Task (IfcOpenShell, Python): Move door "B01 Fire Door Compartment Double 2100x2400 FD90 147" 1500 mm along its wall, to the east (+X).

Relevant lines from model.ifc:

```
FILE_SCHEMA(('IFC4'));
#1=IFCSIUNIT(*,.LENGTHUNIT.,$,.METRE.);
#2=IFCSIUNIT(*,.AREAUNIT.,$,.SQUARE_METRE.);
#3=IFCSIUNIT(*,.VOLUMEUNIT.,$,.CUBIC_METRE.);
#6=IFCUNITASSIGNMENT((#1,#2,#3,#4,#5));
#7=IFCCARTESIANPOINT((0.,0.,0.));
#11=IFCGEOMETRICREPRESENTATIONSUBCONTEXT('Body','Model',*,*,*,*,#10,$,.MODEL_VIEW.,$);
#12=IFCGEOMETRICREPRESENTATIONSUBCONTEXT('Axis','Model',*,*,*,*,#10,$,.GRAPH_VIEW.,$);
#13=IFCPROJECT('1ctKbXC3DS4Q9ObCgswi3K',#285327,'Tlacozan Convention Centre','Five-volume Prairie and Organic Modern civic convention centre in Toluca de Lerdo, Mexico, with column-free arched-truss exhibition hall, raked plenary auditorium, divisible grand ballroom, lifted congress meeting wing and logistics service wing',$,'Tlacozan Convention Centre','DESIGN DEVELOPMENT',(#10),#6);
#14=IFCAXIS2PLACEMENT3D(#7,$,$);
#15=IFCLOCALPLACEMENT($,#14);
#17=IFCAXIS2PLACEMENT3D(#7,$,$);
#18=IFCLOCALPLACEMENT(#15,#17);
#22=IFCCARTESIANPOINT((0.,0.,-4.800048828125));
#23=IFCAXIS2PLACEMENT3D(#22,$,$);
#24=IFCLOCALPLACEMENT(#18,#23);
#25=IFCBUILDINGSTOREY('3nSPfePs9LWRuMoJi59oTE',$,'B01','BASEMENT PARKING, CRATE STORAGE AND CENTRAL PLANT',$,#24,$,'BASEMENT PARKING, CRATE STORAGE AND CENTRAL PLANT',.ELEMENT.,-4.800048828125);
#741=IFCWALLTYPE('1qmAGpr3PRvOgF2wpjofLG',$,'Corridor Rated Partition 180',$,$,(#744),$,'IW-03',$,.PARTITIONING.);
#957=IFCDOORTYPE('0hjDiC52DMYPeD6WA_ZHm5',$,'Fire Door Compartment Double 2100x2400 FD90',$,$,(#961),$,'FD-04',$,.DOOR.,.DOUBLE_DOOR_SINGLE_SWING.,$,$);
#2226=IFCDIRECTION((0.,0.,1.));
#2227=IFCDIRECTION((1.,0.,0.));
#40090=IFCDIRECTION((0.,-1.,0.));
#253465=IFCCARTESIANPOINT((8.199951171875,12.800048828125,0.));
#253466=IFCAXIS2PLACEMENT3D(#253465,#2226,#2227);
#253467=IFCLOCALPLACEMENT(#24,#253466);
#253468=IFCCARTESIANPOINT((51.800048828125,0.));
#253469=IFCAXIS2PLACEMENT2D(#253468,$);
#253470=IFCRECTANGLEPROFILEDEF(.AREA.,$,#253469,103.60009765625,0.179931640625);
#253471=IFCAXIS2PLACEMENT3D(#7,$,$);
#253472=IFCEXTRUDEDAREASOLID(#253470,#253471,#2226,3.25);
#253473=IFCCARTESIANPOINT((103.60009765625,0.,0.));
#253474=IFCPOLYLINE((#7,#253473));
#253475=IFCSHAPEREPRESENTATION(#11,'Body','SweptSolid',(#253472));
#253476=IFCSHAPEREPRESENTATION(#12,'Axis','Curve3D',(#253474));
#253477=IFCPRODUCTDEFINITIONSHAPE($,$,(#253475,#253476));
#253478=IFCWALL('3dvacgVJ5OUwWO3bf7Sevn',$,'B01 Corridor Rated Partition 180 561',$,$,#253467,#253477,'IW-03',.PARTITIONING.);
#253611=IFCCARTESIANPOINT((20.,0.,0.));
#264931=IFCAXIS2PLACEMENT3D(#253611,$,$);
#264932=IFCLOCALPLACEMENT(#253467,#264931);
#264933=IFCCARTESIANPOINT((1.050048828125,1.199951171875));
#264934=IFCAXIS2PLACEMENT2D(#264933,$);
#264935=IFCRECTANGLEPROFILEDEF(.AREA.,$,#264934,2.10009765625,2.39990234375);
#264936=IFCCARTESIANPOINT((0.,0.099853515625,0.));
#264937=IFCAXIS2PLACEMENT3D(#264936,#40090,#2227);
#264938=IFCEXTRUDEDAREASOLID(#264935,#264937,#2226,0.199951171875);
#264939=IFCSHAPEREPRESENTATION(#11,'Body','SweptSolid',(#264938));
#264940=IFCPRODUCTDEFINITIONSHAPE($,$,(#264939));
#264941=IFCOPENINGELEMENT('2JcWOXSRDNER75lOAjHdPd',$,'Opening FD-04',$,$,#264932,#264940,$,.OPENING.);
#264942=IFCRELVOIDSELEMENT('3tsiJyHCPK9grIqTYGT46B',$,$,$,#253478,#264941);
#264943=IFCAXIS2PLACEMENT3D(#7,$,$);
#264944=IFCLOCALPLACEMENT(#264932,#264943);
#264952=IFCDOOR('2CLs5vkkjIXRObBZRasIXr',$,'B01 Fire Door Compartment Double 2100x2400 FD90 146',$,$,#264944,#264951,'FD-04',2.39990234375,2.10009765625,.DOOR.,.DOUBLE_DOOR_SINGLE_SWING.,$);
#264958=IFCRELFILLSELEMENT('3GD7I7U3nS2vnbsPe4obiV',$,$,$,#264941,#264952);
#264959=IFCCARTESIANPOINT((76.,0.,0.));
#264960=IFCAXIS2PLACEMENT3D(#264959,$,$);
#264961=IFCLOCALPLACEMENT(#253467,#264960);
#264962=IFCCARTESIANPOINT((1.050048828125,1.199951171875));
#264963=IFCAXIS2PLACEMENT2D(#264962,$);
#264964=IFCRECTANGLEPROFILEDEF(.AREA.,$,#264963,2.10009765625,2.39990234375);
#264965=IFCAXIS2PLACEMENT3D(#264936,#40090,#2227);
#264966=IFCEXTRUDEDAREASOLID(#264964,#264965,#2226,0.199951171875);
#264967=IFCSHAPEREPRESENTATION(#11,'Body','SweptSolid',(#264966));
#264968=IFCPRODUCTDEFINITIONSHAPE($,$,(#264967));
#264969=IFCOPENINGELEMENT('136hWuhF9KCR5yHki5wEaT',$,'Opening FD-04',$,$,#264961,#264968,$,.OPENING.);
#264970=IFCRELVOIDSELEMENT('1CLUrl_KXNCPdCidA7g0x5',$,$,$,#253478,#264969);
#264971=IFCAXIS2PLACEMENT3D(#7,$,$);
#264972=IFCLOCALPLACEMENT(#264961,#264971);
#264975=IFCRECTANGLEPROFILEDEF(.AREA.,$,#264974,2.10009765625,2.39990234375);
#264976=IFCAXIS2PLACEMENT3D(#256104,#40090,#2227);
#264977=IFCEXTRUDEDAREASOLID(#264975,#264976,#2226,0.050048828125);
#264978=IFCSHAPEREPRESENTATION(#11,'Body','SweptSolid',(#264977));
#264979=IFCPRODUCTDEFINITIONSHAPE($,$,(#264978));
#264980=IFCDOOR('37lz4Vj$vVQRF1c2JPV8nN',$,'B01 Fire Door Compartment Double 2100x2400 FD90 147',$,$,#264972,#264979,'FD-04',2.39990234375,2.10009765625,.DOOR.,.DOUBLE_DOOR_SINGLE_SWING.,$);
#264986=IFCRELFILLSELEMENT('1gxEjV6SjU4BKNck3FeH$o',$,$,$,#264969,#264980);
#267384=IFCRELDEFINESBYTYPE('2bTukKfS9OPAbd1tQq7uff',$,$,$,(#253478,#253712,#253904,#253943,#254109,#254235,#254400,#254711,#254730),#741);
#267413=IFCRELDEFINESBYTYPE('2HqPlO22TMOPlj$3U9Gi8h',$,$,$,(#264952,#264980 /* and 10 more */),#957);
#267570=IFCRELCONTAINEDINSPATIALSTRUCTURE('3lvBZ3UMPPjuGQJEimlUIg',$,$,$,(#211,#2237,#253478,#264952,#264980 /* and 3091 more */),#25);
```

```python
import ifcopenshell
import ifcopenshell.api.geometry
import ifcopenshell.util.placement
import ifcopenshell.util.unit

model = ifcopenshell.open("model.ifc")
unit_scale = ifcopenshell.util.unit.calculate_unit_scale(model)

door = model.by_guid("37lz4Vj$vVQRF1c2JPV8nN")
opening = door.FillsVoids[0].RelatingOpeningElement
wall = opening.VoidsElements[0].RelatingBuildingElement

wall_matrix = ifcopenshell.util.placement.get_local_placement(wall.ObjectPlacement)
shift = wall_matrix[:3, 0] * 1.5 / unit_scale
before = ifcopenshell.util.placement.get_local_placement(door.ObjectPlacement)[:3, 3].copy()

# The door is placed relative to its opening, so it follows when the opening moves.
matrix = ifcopenshell.util.placement.get_local_placement(opening.ObjectPlacement)
matrix[:3, 3] += shift
ifcopenshell.api.geometry.edit_object_placement(
    model, product=opening, matrix=matrix, is_si=False, should_transform_children=True
)

after = ifcopenshell.util.placement.get_local_placement(door.ObjectPlacement)[:3, 3]
print("door moved by", (after - before).round(3) + 0.0)

model.write("model_v2.ifc")
```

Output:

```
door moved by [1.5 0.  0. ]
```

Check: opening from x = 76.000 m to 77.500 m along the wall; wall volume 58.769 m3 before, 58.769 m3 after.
